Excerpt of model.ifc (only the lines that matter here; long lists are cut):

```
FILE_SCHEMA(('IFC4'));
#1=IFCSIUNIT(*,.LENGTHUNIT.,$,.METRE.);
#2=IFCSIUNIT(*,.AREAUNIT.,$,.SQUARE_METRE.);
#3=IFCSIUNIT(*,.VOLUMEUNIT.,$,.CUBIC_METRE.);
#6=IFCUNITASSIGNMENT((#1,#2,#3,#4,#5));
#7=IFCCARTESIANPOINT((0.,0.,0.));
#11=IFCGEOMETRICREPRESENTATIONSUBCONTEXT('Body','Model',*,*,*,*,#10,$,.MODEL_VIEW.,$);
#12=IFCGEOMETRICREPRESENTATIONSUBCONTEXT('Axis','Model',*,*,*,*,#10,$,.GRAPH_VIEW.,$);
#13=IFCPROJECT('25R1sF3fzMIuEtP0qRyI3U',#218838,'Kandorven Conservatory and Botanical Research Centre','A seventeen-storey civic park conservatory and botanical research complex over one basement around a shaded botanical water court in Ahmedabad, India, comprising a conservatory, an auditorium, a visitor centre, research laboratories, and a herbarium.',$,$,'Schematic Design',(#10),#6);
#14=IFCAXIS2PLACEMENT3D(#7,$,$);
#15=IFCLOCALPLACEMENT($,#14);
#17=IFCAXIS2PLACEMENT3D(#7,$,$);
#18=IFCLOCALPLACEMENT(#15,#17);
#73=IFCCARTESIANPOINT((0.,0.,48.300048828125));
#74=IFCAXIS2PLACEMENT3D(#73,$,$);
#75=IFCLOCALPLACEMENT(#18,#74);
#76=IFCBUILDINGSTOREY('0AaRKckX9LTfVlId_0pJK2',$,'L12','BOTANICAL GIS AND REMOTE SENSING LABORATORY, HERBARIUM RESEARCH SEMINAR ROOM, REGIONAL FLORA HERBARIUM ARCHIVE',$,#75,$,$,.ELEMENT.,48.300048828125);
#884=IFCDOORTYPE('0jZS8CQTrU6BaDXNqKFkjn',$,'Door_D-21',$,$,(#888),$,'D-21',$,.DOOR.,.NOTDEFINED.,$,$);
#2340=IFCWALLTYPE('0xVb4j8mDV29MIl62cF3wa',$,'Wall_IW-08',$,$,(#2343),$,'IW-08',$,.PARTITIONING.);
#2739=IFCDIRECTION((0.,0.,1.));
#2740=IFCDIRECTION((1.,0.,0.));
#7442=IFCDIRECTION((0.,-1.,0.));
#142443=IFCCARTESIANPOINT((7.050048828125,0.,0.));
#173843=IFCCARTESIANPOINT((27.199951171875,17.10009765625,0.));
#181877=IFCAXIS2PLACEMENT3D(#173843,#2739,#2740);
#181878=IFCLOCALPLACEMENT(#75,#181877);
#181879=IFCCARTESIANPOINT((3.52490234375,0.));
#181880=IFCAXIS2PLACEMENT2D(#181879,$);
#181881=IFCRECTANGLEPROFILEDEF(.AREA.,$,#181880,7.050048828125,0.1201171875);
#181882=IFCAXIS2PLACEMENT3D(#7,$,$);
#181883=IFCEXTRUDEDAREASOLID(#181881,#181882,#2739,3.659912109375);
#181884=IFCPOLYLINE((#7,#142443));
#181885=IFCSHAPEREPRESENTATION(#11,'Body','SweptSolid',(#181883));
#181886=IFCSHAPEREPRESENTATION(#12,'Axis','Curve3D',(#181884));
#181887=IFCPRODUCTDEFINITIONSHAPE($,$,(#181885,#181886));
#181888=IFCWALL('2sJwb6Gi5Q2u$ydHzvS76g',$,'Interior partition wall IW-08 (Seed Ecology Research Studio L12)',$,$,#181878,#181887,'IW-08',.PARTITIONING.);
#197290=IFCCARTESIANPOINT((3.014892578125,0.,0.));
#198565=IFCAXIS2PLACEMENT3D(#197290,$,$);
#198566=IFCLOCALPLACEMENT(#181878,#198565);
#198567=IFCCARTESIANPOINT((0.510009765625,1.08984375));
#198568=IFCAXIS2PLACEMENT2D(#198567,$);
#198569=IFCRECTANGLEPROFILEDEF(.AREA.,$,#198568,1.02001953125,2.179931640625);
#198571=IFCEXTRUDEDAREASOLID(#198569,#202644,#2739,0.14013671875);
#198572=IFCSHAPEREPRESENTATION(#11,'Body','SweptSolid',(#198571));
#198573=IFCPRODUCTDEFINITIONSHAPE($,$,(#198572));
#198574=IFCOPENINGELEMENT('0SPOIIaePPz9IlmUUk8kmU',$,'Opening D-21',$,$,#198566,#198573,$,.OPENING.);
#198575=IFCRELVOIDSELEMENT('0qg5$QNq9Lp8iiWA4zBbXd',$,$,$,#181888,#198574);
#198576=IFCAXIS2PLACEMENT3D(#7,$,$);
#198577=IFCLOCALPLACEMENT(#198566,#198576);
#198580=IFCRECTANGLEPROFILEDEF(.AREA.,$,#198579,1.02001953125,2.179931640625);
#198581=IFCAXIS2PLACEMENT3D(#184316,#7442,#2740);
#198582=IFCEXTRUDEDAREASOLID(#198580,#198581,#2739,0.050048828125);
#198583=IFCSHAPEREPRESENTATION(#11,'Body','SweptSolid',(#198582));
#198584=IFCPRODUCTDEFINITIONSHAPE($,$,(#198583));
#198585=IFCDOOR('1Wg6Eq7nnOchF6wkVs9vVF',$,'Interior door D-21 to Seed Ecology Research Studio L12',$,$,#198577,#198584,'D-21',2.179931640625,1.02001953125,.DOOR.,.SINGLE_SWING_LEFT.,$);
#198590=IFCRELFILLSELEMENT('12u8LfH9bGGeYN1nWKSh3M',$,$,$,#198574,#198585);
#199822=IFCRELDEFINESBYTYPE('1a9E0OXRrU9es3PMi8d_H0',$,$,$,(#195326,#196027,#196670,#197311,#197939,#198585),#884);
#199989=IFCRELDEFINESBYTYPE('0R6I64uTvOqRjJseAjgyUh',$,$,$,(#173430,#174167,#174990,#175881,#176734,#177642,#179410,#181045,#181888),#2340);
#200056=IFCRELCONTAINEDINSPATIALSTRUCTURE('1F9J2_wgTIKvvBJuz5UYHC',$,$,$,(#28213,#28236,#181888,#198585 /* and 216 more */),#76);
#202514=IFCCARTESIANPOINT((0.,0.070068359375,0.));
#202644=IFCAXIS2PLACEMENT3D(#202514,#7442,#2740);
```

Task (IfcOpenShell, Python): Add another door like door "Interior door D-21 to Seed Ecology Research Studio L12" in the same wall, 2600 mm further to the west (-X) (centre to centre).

```python
import ifcopenshell
import ifcopenshell.api.feature
import ifcopenshell.api.geometry
import ifcopenshell.api.root
import ifcopenshell.geom
import ifcopenshell.util.element
import ifcopenshell.util.placement
import ifcopenshell.util.shape
import ifcopenshell.util.unit

model = ifcopenshell.open("model.ifc")
unit_scale = ifcopenshell.util.unit.calculate_unit_scale(model)
settings = ifcopenshell.geom.settings()


def volume(element):
    """Net volume in cubic metres, openings subtracted."""
    shape = ifcopenshell.geom.create_shape(settings, element)
    return ifcopenshell.util.shape.get_volume(shape.geometry)


door = model.by_guid("1Wg6Eq7nnOchF6wkVs9vVF")
opening = door.FillsVoids[0].RelatingOpeningElement
wall = opening.VoidsElements[0].RelatingBuildingElement
before = volume(wall)
shift = ifcopenshell.util.placement.get_local_placement(wall.ObjectPlacement)[:3, 0] * -2.6 / unit_scale

# copy_class copies the void relationship, type, container and properties, but no geometry.
new_opening = ifcopenshell.api.root.copy_class(model, product=opening)
new_opening.Representation = ifcopenshell.util.element.copy_deep(
    model, opening.Representation, exclude=["IfcGeometricRepresentationContext", "IfcRepresentationMap"]
)
new_door = ifcopenshell.api.root.copy_class(model, product=door)
new_door.Representation = ifcopenshell.util.element.copy_deep(
    model, door.Representation, exclude=["IfcGeometricRepresentationContext", "IfcRepresentationMap"]
)
new_door.Tag = None
ifcopenshell.api.feature.add_filling(model, opening=new_opening, element=new_door)

for old, new in ((opening, new_opening), (door, new_door)):
    matrix = ifcopenshell.util.placement.get_local_placement(old.ObjectPlacement)
    matrix[:3, 3] += shift
    ifcopenshell.api.geometry.edit_object_placement(model, product=new, matrix=matrix, is_si=False)

after = volume(wall)

print(f"wall volume {before:.3f} -> {after:.3f} m3")

model.write("model-out.ifc")
```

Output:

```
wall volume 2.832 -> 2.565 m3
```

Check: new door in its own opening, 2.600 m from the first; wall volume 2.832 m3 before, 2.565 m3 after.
